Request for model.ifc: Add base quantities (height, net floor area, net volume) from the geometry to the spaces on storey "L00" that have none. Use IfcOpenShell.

First a look at what the model holds.

```python
import ifcopenshell
import ifcopenshell.util.element
import ifcopenshell.util.unit

model = ifcopenshell.open("model.ifc")
print(model.schema)
for unit_type in ("LENGTHUNIT", "AREAUNIT", "VOLUMEUNIT"):
    print(unit_type, ifcopenshell.util.unit.calculate_unit_scale(model, unit_type))
storey = next(s for s in model.by_type("IfcBuildingStorey") if s.Name == "L00")
spaces = [e for e in ifcopenshell.util.element.get_decomposition(storey) if e.is_a("IfcSpace")]
for e in sorted(spaces, key=lambda e: e.id()):
    print(e.id(), e.is_a(), e.Name, list(ifcopenshell.util.element.get_psets(e, qtos_only=True)), sep=" | ")
```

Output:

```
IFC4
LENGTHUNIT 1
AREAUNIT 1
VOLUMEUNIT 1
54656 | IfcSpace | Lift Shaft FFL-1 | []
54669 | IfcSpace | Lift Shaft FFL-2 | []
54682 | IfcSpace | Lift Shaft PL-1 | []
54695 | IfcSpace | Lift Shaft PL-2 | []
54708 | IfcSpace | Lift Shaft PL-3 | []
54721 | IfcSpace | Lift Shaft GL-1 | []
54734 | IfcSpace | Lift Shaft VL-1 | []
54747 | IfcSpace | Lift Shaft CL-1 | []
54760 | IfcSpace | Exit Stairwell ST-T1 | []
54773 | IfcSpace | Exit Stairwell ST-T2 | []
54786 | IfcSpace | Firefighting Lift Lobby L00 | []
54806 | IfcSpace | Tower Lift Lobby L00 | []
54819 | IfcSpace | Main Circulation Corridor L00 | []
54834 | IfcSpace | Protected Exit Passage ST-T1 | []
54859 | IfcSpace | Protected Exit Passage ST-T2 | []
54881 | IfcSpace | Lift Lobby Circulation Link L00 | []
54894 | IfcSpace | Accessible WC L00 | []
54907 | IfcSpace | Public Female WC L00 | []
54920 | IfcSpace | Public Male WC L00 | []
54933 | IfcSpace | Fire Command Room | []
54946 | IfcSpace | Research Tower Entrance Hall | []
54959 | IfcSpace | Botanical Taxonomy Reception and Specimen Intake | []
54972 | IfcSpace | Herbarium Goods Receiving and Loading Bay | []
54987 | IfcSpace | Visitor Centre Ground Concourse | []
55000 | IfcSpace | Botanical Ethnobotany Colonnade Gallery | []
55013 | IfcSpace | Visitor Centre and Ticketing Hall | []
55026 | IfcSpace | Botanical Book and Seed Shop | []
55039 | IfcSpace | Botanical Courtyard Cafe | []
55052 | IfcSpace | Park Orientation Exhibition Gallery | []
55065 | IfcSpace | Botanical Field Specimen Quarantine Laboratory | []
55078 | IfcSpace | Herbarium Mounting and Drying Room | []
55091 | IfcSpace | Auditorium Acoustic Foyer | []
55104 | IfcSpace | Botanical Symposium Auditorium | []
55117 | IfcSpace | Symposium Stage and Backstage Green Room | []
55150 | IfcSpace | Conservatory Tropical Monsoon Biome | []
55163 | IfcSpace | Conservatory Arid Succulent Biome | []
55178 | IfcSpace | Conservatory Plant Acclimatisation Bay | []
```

```python
import ifcopenshell
import ifcopenshell.api.pset
import ifcopenshell.geom
import ifcopenshell.util.element
import ifcopenshell.util.shape
import ifcopenshell.util.unit

model = ifcopenshell.open("model.ifc")
unit_scale = ifcopenshell.util.unit.calculate_unit_scale(model)
area_scale = ifcopenshell.util.unit.calculate_unit_scale(model, "AREAUNIT")
volume_scale = ifcopenshell.util.unit.calculate_unit_scale(model, "VOLUMEUNIT")
settings = ifcopenshell.geom.settings()

storey = next(s for s in model.by_type("IfcBuildingStorey") if s.Name == "L00")
spaces = [e for e in ifcopenshell.util.element.get_decomposition(storey) if e.is_a("IfcSpace")]

for e in sorted(spaces, key=lambda e: e.id()):
    if ifcopenshell.util.element.get_psets(e, qtos_only=True, should_inherit=False):
        continue
    # Geometry comes back in metres, in the element's own axes.
    shape = ifcopenshell.geom.create_shape(settings, e)
    values = {
        "Height": ifcopenshell.util.shape.get_z(shape.geometry) / unit_scale,
        "NetFloorArea": ifcopenshell.util.shape.get_footprint_area(shape.geometry) / area_scale,
        "NetVolume": ifcopenshell.util.shape.get_volume(shape.geometry) / volume_scale,
    }
    qto = ifcopenshell.api.pset.add_qto(model, product=e, name="Qto_SpaceBaseQuantities")
    ifcopenshell.api.pset.edit_qto(model, qto=qto, properties=values)
    print(e.id(), {k: round(v, 3) for k, v in values.items()})

model.write("model_v2.ifc")
```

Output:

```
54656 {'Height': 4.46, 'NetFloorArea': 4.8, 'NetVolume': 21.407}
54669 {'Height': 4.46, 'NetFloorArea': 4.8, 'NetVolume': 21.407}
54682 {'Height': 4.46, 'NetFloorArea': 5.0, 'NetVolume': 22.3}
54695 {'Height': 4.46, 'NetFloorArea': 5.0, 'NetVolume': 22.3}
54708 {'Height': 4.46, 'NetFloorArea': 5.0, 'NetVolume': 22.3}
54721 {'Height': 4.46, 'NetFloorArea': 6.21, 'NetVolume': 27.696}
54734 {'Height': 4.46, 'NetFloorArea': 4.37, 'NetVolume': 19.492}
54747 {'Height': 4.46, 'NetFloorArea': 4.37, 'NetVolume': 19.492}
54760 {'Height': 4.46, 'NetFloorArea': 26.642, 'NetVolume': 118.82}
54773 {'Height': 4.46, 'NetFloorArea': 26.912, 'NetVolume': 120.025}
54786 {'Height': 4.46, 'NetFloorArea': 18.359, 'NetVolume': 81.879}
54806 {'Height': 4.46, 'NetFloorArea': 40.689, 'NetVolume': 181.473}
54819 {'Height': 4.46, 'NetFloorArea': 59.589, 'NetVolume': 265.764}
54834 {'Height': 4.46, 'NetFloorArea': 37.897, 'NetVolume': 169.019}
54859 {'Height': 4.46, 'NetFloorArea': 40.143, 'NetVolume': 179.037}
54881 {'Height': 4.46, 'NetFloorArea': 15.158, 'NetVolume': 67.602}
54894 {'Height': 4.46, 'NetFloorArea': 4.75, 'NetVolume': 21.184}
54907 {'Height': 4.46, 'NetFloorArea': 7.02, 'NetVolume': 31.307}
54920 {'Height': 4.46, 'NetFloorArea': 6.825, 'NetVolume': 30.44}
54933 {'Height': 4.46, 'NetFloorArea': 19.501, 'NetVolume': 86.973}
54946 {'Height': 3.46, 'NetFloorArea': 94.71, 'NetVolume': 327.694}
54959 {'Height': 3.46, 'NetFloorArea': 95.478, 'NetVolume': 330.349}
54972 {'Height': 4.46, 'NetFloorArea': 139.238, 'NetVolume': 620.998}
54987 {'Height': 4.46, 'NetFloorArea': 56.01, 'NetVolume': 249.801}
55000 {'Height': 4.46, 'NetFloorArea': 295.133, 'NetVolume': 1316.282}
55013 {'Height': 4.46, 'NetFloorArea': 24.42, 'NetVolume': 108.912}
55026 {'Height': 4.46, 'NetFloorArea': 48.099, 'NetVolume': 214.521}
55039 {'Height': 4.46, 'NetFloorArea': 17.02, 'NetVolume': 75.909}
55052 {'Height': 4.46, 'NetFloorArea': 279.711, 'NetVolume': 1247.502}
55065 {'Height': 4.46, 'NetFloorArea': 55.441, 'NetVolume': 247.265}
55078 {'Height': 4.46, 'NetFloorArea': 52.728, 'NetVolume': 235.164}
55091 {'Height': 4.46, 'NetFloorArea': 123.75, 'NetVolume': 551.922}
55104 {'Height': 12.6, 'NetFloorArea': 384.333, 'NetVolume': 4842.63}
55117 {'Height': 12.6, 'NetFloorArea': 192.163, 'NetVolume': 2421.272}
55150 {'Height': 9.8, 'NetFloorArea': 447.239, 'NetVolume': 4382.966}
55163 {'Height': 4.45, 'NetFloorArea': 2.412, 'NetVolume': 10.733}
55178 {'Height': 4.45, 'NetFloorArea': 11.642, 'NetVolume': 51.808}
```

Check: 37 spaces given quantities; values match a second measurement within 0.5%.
